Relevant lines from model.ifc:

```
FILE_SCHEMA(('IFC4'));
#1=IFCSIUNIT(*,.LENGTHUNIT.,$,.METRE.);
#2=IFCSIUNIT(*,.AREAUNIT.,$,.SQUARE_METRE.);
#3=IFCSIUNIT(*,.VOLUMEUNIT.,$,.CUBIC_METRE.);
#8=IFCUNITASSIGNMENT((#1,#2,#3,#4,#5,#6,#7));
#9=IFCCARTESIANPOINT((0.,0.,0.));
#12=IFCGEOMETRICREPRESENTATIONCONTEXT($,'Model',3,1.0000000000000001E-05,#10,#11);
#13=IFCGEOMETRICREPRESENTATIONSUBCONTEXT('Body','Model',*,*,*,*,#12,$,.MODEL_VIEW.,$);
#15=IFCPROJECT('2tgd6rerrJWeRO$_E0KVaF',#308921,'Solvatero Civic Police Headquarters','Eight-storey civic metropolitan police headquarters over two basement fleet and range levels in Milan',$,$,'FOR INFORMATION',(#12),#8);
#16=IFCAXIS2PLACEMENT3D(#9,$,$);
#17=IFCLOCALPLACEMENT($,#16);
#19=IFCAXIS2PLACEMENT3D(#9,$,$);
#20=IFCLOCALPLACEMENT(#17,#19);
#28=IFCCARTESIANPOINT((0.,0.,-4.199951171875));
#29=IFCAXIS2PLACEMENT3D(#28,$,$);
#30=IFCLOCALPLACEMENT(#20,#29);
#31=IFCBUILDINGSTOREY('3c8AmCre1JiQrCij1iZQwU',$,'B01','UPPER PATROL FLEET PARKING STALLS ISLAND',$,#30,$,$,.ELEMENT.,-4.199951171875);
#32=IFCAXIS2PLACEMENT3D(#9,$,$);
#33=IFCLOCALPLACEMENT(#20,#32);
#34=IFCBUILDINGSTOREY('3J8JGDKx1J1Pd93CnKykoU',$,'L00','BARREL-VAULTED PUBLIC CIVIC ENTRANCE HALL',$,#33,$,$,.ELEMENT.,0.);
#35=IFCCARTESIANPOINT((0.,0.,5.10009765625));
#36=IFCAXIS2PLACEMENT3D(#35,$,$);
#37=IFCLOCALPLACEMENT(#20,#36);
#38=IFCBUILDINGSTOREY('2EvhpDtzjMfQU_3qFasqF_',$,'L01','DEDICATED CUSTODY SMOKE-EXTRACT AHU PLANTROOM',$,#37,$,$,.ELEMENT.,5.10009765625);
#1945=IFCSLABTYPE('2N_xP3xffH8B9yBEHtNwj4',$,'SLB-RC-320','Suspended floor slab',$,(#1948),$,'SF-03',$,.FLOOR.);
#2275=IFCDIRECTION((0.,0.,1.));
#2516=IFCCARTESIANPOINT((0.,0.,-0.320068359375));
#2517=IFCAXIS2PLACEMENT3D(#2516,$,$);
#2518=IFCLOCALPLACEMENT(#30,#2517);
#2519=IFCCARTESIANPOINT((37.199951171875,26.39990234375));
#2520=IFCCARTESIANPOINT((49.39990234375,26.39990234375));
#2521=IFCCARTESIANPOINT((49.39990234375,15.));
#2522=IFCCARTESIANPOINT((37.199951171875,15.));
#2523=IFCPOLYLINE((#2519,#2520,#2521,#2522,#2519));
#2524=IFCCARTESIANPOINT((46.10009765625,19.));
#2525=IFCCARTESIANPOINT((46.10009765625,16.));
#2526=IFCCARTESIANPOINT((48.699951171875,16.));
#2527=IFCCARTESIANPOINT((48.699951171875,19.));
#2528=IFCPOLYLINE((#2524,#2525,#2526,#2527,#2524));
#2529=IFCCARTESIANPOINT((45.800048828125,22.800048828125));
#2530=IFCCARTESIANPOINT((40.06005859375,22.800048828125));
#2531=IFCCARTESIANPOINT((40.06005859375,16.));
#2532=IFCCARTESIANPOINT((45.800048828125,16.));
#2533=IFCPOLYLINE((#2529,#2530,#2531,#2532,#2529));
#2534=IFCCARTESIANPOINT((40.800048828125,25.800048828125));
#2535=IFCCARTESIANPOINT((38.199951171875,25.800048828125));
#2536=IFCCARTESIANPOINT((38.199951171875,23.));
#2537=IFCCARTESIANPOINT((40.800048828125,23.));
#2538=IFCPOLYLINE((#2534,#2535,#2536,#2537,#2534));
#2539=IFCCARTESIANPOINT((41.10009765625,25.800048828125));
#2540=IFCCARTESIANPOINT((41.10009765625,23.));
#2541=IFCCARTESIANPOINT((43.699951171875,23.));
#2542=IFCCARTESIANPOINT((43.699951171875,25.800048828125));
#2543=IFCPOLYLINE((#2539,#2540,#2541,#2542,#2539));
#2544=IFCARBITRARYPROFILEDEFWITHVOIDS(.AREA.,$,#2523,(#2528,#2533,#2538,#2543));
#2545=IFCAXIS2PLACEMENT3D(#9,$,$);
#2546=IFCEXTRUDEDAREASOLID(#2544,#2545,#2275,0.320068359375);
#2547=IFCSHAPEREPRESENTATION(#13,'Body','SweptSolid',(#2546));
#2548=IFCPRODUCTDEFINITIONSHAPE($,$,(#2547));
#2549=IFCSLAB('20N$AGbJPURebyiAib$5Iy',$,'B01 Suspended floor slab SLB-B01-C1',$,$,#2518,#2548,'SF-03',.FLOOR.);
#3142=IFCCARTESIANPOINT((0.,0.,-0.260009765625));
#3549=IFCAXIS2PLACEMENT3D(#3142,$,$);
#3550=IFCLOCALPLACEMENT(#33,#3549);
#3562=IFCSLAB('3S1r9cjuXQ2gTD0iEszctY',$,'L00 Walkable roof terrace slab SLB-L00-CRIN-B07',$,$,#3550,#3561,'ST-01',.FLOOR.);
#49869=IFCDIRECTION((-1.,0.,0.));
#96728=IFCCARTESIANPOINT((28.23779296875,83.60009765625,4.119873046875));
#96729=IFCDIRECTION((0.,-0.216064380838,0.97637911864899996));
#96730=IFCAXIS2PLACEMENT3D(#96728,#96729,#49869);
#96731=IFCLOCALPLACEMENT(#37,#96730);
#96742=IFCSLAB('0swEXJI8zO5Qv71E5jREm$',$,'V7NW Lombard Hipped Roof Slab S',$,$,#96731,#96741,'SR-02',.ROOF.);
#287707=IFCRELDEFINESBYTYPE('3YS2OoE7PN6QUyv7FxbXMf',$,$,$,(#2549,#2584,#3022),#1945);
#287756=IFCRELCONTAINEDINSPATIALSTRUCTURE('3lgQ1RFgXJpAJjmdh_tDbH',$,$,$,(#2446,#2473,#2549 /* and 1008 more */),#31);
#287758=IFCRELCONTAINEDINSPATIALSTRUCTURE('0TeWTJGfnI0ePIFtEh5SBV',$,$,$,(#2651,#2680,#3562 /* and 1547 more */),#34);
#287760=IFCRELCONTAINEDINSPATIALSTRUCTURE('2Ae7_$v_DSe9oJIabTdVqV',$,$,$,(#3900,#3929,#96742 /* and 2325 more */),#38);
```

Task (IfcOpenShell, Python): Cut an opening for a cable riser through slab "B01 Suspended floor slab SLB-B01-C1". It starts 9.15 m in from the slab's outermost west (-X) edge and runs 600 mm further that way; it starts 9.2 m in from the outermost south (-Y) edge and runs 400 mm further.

```python
import numpy as np
import ifcopenshell
import ifcopenshell.api.feature
import ifcopenshell.api.geometry
import ifcopenshell.api.root
import ifcopenshell.geom
import ifcopenshell.util.placement
import ifcopenshell.util.representation
import ifcopenshell.util.shape
import ifcopenshell.util.unit

model = ifcopenshell.open("model.ifc")
unit_scale = ifcopenshell.util.unit.calculate_unit_scale(model)
settings = ifcopenshell.geom.settings()


def volume(element):
    """Net volume in cubic metres, openings subtracted."""
    shape = ifcopenshell.geom.create_shape(settings, element)
    return ifcopenshell.util.shape.get_volume(shape.geometry)


slab = model.by_id(2549)
before = volume(slab)

# Extent in the slab's own axes, in metres. The edges named are its -X and -Y sides.
slab_shape = ifcopenshell.geom.create_shape(settings, slab)
vertices = ifcopenshell.util.shape.get_vertices(slab_shape.geometry)
x_min, y_min, bottom = vertices.min(axis=0)
top = vertices[:, 2].max()

opening = ifcopenshell.api.root.create_entity(model, ifc_class="IfcOpeningElement", name="Cable riser opening", predefined_type="OPENING")
context = ifcopenshell.util.representation.get_context(model, "Model", "Body", "MODEL_VIEW")
width, depth = 0.6, 0.4
outline = [(0.0, 0.0), (width, 0.0), (width, depth), (0.0, depth), (0.0, 0.0)]
# Overshoot both faces by 50 mm so the cut is clean.
shape = ifcopenshell.api.geometry.add_slab_representation(
    model, context=context, depth=top - bottom + 0.1, polyline=outline
)
ifcopenshell.api.geometry.assign_representation(model, product=opening, representation=shape)

matrix = ifcopenshell.util.placement.get_local_placement(slab.ObjectPlacement)
matrix[:, 3] = matrix @ np.append(np.array([x_min + 9.15, y_min + 9.2, bottom - 0.05]) / unit_scale, 1.0)
ifcopenshell.api.geometry.edit_object_placement(model, product=opening, matrix=matrix, is_si=False)
ifcopenshell.api.feature.add_feature(model, feature=opening, element=slab)

after = volume(slab)

print(f"slab volume {before:.3f} -> {after:.3f} m3")

model.write("model_edited.ifc")
```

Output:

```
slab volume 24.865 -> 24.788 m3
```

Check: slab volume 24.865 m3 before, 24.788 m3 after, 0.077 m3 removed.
